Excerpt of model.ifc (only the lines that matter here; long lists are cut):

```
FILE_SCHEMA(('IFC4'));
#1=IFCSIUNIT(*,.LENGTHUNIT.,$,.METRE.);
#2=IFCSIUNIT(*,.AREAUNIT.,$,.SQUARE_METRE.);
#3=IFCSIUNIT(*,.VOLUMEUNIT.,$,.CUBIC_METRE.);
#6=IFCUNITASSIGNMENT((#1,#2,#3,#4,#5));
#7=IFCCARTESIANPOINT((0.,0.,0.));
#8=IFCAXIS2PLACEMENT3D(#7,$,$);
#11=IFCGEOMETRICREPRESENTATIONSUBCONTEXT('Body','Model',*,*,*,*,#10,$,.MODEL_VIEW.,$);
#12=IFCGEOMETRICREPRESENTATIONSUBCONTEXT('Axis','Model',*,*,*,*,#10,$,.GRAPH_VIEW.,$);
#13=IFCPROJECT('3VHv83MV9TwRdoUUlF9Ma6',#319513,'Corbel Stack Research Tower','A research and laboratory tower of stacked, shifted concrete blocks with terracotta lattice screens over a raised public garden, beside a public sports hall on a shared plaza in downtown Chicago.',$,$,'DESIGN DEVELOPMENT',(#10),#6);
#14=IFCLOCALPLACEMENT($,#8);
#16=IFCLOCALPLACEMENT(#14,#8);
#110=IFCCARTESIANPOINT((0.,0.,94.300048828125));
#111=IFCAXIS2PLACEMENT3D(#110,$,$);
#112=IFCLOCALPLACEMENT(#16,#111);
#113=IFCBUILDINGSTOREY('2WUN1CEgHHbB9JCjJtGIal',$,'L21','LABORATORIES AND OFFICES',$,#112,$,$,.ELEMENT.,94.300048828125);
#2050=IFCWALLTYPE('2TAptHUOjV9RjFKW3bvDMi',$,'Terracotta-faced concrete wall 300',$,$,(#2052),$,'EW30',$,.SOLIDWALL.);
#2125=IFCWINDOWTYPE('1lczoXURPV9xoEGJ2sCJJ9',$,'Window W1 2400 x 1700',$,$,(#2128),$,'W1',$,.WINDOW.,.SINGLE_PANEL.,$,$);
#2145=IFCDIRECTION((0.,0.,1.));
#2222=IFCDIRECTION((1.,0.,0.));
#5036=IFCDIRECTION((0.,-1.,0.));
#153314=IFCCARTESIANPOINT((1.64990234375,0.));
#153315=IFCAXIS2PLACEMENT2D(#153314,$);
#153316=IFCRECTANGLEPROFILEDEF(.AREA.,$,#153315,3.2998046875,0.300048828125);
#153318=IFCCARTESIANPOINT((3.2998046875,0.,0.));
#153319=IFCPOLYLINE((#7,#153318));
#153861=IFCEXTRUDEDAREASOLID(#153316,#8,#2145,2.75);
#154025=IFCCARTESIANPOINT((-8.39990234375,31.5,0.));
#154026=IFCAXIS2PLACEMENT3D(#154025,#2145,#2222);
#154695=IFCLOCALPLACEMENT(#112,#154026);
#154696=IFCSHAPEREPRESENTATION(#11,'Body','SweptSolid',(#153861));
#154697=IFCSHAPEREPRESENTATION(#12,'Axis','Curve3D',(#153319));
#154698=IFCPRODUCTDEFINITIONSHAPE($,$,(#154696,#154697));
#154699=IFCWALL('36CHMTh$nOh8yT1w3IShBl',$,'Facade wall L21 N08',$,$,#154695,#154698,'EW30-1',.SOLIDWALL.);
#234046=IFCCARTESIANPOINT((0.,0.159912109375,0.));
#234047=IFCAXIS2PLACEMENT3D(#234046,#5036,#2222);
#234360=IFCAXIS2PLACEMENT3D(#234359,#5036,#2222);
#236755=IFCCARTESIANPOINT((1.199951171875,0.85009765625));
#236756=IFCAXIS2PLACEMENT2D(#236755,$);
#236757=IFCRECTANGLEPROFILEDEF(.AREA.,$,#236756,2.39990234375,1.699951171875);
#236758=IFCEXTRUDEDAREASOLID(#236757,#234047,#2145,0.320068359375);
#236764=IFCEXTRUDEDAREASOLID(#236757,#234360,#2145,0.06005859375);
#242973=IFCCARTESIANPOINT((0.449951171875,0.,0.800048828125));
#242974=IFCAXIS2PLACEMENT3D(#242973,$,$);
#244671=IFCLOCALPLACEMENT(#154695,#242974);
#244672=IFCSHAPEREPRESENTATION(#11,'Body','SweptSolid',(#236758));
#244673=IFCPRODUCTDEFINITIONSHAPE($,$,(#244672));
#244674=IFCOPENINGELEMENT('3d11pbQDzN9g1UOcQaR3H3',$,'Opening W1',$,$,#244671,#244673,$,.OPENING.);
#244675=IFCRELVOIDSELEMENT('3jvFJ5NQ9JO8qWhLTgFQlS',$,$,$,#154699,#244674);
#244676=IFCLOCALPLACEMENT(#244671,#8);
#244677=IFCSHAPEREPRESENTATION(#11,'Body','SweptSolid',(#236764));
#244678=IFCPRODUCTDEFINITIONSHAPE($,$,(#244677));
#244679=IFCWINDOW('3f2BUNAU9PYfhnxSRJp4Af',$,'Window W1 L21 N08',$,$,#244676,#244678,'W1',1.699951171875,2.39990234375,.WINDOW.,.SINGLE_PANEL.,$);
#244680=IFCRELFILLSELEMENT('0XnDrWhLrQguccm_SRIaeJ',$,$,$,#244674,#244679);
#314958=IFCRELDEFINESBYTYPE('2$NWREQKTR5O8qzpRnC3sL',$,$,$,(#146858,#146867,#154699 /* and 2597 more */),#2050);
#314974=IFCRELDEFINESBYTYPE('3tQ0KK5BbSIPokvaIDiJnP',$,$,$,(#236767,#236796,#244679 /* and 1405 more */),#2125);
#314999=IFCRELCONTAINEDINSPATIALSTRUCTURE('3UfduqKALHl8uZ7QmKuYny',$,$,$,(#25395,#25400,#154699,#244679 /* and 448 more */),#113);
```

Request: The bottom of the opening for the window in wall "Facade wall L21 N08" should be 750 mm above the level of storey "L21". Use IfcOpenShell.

```python
import numpy as np
import ifcopenshell
import ifcopenshell.api.geometry
import ifcopenshell.geom
import ifcopenshell.util.element
import ifcopenshell.util.placement
import ifcopenshell.util.shape
import ifcopenshell.util.unit

model = ifcopenshell.open("model.ifc")
unit_scale = ifcopenshell.util.unit.calculate_unit_scale(model)

window = model.by_id(244679)
opening = window.FillsVoids[0].RelatingOpeningElement
storey = ifcopenshell.util.element.get_container(window, ifc_class="IfcBuildingStorey")
level = ifcopenshell.util.placement.get_local_placement(storey.ObjectPlacement)[2, 3]

# The opening's origin need not be at the sill, so measure its lowest point.
shape = ifcopenshell.geom.create_shape(ifcopenshell.geom.settings(), opening)
bottom = ifcopenshell.util.shape.get_shape_bottom_elevation(shape, shape.geometry) / unit_scale
dz = level + 0.75 / unit_scale - bottom

shift = np.array([0.0, 0.0, dz])
# The window is placed relative to its opening, so it follows when the opening moves.
matrix = ifcopenshell.util.placement.get_local_placement(opening.ObjectPlacement)
matrix[:3, 3] += shift
ifcopenshell.api.geometry.edit_object_placement(
    model, product=opening, matrix=matrix, is_si=False, should_transform_children=True
)

print(f"moved by {dz * unit_scale:+.3f} m")

model.write("model_edited.ifc")
```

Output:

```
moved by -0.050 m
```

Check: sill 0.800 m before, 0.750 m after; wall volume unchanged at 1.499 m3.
